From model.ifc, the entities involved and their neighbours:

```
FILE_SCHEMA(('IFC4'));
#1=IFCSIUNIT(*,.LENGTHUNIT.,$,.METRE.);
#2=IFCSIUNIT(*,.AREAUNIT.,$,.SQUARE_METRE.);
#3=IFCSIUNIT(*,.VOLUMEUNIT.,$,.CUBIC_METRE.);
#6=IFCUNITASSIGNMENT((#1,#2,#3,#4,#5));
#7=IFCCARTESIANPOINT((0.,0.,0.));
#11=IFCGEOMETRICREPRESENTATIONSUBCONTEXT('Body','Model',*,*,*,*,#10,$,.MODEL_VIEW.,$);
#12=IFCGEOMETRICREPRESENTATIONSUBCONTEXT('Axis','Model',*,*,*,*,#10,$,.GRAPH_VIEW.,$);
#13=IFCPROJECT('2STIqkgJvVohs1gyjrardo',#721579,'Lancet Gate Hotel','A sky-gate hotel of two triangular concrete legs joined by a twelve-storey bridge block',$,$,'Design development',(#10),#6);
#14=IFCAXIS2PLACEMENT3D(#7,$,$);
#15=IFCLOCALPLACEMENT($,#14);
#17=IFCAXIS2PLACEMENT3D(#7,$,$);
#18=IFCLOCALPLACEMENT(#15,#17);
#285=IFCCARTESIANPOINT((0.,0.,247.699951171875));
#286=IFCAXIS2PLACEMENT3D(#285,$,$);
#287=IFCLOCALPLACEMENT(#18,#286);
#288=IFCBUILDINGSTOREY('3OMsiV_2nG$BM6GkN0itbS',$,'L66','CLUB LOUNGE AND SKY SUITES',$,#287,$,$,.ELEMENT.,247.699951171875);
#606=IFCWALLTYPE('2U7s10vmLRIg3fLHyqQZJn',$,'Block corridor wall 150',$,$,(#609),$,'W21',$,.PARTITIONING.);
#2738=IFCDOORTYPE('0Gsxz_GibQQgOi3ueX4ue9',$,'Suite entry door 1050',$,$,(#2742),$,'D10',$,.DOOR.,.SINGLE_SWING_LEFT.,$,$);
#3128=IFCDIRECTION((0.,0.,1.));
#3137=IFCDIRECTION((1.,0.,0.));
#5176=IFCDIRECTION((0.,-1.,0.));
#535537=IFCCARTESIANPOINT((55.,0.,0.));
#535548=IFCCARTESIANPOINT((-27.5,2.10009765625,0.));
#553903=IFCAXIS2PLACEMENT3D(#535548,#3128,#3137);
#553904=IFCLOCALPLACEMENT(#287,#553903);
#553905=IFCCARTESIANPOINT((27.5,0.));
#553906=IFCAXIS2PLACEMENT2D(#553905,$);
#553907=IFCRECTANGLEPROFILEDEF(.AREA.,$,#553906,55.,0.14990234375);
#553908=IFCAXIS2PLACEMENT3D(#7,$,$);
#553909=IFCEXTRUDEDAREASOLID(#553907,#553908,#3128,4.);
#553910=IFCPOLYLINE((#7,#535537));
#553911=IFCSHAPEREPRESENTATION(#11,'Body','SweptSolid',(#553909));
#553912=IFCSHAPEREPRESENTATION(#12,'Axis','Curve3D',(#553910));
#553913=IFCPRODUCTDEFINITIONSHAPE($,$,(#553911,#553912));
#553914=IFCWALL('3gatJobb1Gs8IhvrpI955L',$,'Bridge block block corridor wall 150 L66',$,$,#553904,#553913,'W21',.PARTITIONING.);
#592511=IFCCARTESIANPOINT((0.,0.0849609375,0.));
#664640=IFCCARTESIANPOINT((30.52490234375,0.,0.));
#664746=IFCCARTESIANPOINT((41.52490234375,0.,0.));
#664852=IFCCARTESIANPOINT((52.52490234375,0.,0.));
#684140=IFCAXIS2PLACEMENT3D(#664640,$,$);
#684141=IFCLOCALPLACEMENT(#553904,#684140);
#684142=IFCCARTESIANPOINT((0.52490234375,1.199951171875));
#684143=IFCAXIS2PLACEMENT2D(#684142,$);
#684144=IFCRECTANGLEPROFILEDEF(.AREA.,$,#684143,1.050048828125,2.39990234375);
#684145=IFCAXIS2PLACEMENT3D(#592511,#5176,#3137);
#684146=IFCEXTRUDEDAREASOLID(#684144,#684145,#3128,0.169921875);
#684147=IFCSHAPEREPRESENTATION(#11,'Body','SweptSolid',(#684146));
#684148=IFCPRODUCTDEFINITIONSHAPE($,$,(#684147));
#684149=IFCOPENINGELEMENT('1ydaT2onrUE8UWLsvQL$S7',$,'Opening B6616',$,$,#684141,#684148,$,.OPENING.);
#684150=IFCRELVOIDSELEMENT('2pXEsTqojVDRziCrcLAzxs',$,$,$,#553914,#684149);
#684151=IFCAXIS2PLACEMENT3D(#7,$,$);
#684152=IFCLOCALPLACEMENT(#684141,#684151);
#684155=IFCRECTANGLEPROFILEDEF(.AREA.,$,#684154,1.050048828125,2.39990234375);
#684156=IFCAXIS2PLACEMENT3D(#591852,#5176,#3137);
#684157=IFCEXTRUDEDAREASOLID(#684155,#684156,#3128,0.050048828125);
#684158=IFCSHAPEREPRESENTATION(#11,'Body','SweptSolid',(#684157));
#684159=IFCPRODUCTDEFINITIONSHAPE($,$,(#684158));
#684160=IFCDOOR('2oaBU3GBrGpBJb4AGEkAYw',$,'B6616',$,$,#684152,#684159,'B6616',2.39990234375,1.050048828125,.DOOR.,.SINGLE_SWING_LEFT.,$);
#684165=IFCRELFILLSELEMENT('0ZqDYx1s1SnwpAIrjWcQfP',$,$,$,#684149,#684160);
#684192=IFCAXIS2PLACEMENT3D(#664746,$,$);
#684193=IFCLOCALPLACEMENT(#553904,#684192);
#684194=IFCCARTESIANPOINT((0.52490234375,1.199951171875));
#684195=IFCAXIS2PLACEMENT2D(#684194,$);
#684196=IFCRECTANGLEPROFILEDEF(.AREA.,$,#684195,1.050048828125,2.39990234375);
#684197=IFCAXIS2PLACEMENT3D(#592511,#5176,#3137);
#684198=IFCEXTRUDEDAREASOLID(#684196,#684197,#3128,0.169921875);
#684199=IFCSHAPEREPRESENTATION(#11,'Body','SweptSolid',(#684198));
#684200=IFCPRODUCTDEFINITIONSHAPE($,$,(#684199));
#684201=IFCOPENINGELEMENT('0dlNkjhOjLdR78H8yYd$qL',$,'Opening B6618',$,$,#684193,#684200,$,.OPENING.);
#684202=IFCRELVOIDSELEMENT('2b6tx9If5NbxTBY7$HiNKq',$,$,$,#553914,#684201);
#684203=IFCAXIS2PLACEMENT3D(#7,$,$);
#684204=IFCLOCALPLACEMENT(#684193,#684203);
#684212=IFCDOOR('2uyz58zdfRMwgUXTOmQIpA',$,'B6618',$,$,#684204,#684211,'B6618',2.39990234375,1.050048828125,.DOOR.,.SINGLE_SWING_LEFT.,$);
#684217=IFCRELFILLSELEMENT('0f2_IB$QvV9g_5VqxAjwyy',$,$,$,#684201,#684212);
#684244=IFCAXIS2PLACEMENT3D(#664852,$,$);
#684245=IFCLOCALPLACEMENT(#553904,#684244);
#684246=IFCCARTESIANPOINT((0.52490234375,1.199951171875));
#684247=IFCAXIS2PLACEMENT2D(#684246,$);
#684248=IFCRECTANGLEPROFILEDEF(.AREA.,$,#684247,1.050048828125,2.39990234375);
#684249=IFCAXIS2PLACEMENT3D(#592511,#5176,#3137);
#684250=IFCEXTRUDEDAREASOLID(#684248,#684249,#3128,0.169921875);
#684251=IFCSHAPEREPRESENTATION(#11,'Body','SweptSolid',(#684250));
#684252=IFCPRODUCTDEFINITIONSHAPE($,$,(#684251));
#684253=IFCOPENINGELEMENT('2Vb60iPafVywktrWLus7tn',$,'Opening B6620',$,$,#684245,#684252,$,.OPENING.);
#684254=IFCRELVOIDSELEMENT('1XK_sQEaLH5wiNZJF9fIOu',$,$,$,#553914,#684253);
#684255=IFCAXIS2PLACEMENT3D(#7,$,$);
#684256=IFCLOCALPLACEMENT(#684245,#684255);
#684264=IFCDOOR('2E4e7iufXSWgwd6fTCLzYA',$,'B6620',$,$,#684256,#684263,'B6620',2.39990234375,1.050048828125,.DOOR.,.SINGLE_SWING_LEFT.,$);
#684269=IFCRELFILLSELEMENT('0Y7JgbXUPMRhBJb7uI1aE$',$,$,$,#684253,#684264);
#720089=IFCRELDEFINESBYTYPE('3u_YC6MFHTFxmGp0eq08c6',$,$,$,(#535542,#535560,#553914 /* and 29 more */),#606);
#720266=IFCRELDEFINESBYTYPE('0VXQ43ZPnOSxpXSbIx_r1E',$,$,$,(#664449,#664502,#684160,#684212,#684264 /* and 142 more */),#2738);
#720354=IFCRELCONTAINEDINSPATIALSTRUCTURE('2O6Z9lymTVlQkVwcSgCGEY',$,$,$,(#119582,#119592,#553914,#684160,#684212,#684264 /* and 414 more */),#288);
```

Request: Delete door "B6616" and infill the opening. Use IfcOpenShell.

```python
import ifcopenshell
import ifcopenshell.api.feature
import ifcopenshell.api.root
import ifcopenshell.geom
import ifcopenshell.util.shape

model = ifcopenshell.open("model.ifc")
settings = ifcopenshell.geom.settings()


def volume(element):
    """Net volume in cubic metres, openings subtracted."""
    shape = ifcopenshell.geom.create_shape(settings, element)
    return ifcopenshell.util.shape.get_volume(shape.geometry)


door = model.by_guid("2oaBU3GBrGpBJb4AGEkAYw")
opening = door.FillsVoids[0].RelatingOpeningElement
wall = opening.VoidsElements[0].RelatingBuildingElement
before = volume(wall)

ifcopenshell.api.root.remove_product(model, product=door)
ifcopenshell.api.feature.remove_feature(model, feature=opening)

after = volume(wall)

print(f"wall volume {before:.3f} -> {after:.3f} m3")

model.write("model_edited.ifc")
```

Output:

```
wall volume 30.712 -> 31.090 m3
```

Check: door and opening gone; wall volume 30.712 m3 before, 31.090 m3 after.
